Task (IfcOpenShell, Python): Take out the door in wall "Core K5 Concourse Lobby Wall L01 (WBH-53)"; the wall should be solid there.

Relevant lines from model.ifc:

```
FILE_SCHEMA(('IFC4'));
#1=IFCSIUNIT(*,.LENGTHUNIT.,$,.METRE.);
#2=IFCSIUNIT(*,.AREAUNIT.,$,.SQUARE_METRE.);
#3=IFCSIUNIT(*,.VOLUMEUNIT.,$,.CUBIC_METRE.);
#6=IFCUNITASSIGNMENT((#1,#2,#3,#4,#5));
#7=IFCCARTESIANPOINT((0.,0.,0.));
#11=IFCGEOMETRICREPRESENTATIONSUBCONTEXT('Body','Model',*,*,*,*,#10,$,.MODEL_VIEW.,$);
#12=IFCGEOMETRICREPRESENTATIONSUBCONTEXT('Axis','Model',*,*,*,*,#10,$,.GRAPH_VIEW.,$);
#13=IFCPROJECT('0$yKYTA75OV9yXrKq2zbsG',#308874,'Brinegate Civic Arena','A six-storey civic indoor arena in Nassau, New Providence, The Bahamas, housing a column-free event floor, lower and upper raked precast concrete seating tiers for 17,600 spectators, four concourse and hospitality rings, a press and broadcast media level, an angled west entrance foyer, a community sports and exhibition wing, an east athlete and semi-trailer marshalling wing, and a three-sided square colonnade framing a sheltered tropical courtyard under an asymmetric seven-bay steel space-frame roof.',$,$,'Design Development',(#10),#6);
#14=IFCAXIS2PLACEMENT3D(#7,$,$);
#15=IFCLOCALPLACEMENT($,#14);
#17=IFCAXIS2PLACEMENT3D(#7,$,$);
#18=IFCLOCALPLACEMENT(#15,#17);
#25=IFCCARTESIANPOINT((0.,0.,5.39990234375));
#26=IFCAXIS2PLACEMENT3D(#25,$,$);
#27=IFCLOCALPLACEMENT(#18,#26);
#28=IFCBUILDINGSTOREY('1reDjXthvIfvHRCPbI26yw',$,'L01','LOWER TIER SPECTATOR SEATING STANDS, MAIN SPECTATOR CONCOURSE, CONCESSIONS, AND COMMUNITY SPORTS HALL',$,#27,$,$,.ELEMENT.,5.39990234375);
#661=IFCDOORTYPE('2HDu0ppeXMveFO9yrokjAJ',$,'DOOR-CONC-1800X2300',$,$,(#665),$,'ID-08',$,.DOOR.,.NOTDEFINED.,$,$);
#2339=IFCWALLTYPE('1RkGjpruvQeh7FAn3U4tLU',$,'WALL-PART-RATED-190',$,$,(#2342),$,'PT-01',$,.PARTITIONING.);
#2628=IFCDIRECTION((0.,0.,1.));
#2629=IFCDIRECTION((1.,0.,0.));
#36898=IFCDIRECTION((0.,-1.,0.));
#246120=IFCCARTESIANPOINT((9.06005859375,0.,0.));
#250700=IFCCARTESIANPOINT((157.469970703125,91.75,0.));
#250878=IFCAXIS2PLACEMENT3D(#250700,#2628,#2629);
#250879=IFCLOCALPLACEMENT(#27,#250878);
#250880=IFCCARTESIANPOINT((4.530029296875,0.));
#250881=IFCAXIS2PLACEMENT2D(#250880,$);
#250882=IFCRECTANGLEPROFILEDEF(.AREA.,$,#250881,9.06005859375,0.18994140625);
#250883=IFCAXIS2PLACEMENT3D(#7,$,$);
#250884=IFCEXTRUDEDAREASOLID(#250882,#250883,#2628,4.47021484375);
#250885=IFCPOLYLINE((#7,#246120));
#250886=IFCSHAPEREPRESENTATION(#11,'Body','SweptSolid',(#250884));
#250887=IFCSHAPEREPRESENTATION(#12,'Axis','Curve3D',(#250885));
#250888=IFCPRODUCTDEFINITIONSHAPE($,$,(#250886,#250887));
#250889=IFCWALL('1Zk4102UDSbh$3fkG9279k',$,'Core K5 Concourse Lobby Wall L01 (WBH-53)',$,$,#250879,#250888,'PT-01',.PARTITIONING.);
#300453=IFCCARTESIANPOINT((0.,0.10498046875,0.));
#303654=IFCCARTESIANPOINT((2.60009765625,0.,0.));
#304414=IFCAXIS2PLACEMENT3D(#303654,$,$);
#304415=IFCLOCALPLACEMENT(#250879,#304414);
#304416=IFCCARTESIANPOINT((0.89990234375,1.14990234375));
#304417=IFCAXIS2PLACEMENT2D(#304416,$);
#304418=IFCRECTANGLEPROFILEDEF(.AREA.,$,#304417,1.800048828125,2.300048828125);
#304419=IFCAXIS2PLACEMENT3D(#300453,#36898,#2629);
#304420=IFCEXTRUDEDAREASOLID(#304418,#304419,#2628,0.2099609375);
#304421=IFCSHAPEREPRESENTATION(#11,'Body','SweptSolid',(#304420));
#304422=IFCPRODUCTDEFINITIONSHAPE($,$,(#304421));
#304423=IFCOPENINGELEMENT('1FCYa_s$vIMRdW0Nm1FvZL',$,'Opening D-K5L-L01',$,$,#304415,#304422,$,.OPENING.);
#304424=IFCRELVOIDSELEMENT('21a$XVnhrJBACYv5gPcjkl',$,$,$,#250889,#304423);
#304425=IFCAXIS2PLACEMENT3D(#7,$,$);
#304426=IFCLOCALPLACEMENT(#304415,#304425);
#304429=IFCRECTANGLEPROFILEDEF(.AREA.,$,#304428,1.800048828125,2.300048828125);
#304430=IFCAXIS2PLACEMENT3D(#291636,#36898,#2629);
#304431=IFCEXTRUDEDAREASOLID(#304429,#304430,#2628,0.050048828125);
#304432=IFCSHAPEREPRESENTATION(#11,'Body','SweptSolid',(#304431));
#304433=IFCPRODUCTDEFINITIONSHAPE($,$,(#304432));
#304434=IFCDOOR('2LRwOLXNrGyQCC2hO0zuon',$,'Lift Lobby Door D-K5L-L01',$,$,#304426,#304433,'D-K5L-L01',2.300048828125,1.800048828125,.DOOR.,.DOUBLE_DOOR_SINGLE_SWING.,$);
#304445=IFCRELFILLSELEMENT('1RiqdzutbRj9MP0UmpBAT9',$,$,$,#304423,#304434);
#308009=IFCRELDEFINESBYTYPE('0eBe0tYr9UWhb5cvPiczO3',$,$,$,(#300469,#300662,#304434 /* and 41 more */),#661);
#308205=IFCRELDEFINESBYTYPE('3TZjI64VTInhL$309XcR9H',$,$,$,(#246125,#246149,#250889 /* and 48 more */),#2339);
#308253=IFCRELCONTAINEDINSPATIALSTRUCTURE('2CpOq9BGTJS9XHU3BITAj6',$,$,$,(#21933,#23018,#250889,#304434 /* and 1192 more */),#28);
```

```python
import ifcopenshell
import ifcopenshell.api.feature
import ifcopenshell.api.root
import ifcopenshell.geom
import ifcopenshell.util.shape

model = ifcopenshell.open("model.ifc")
settings = ifcopenshell.geom.settings()


def volume(element):
    """Net volume in cubic metres, openings subtracted."""
    shape = ifcopenshell.geom.create_shape(settings, element)
    return ifcopenshell.util.shape.get_volume(shape.geometry)


door = model.by_id(304434)
opening = door.FillsVoids[0].RelatingOpeningElement
wall = opening.VoidsElements[0].RelatingBuildingElement
before = volume(wall)

ifcopenshell.api.root.remove_product(model, product=door)
ifcopenshell.api.feature.remove_feature(model, feature=opening)

after = volume(wall)

print(f"wall volume {before:.3f} -> {after:.3f} m3")

model.write("model_v2.ifc")
```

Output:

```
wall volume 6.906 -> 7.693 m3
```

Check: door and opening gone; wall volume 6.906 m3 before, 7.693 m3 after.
